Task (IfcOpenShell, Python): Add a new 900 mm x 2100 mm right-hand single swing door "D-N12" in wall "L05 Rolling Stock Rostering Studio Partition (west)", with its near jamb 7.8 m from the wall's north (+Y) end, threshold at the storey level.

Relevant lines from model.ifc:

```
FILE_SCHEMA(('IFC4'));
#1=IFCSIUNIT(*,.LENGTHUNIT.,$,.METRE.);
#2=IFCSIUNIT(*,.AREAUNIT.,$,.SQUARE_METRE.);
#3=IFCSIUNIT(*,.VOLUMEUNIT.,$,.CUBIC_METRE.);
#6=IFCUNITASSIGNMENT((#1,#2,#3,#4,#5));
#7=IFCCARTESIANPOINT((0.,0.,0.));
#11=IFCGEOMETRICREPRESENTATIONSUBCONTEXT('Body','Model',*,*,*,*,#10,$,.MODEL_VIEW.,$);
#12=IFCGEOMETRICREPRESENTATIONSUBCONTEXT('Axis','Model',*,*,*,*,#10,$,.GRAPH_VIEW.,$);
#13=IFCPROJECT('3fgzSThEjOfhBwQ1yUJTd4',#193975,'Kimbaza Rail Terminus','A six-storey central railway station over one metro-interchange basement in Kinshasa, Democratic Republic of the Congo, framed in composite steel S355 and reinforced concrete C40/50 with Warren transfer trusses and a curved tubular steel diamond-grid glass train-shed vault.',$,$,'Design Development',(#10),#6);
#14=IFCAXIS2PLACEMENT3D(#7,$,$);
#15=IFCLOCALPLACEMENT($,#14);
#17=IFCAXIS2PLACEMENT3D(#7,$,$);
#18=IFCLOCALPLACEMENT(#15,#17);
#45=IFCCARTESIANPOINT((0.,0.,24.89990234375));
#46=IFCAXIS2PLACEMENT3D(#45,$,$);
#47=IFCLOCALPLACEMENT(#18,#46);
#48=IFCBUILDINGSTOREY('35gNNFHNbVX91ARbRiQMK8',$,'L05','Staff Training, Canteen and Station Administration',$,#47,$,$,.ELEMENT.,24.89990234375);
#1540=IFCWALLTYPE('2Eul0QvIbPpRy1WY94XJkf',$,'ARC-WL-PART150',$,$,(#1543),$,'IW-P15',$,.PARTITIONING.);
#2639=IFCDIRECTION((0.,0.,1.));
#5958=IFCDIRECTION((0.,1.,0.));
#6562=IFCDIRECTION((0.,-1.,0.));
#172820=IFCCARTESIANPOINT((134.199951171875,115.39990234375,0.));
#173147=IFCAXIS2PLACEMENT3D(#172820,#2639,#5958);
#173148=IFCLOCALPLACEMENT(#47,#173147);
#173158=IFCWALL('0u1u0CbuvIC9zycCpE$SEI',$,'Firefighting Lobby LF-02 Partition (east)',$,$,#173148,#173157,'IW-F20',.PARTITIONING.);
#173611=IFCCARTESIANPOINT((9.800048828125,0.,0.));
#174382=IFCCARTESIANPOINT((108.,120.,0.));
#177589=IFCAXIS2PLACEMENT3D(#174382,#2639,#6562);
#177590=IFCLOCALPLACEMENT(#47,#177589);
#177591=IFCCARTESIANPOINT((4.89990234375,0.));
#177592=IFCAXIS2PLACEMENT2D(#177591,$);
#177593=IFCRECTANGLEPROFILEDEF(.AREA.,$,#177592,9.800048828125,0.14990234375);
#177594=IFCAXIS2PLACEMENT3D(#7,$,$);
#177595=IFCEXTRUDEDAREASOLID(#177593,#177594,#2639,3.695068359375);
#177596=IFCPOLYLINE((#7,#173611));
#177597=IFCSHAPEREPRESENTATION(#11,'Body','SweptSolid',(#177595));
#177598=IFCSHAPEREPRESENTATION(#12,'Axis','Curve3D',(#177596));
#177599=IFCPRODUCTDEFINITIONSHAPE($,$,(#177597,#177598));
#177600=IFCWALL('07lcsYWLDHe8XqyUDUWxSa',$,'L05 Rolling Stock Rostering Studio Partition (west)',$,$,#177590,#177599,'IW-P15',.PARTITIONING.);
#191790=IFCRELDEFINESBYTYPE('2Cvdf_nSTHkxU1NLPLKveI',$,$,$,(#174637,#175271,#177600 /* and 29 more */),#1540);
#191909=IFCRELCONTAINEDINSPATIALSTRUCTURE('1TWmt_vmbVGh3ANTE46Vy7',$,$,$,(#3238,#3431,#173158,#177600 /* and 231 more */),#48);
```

```python
import numpy as np
import ifcopenshell
import ifcopenshell.api.feature
import ifcopenshell.api.geometry
import ifcopenshell.api.root
import ifcopenshell.api.spatial
import ifcopenshell.geom
import ifcopenshell.util.element
import ifcopenshell.util.placement
import ifcopenshell.util.representation
import ifcopenshell.util.shape
import ifcopenshell.util.unit

model = ifcopenshell.open("model.ifc")
unit_scale = ifcopenshell.util.unit.calculate_unit_scale(model)
settings = ifcopenshell.geom.settings()


def volume(element):
    """Net volume in cubic metres, openings subtracted."""
    shape = ifcopenshell.geom.create_shape(settings, element)
    return ifcopenshell.util.shape.get_volume(shape.geometry)


wall = model.by_guid("07lcsYWLDHe8XqyUDUWxSa")
storey = ifcopenshell.util.element.get_container(wall, ifc_class="IfcBuildingStorey")
context = ifcopenshell.util.representation.get_context(model, "Model", "Body", "MODEL_VIEW")
before = volume(wall)

width, height, from_end, sill = 0.9, 2.1, 7.8, 0.0  # metres

# The wall runs along its own X axis, and the end named is its -X end.
wall_shape = ifcopenshell.geom.create_shape(settings, wall)
x, y, z = ifcopenshell.util.shape.get_vertices(wall_shape.geometry).T
start = x.min() + from_end
face, thickness = float(y.min()), float(y.max() - y.min())
wall_matrix = ifcopenshell.util.placement.get_local_placement(wall.ObjectPlacement)
level = ifcopenshell.util.placement.get_local_placement(storey.ObjectPlacement)[2, 3]


def in_wall(x, y):
    """Placement at x, y metres in the wall's axes, at sill height."""
    matrix = wall_matrix.copy()
    matrix[:, 3] = wall_matrix @ np.array([x / unit_scale, y / unit_scale, 0.0, 1.0])
    matrix[2, 3] = level + sill / unit_scale
    return matrix


# Opening: a box that overshoots both wall faces by 50 mm.
opening = ifcopenshell.api.root.create_entity(model, ifc_class="IfcOpeningElement", predefined_type="OPENING")
box = ifcopenshell.api.geometry.add_wall_representation(
    model, context=context, length=width, height=height, thickness=thickness + 0.1
)
ifcopenshell.api.geometry.assign_representation(model, product=opening, representation=box)
ifcopenshell.api.geometry.edit_object_placement(model, product=opening, matrix=in_wall(start, face - 0.05), is_si=False)
ifcopenshell.api.feature.add_feature(model, feature=opening, element=wall)

door = ifcopenshell.api.root.create_entity(model, ifc_class="IfcDoor", name="D-N12", predefined_type="DOOR")
door.OverallWidth, door.OverallHeight = width / unit_scale, height / unit_scale
door.OperationType = "SINGLE_SWING_RIGHT"
body = ifcopenshell.api.geometry.add_door_representation(
    model,
    context=context,
    overall_width=door.OverallWidth,
    overall_height=door.OverallHeight,
    operation_type="SINGLE_SWING_RIGHT",
    lining_properties={"LiningDepth": thickness / unit_scale, "ThresholdDepth": thickness / unit_scale},
)
ifcopenshell.api.geometry.assign_representation(model, product=door, representation=body)
ifcopenshell.api.spatial.assign_container(model, products=[door], relating_structure=storey)
ifcopenshell.api.feature.add_filling(model, opening=opening, element=door)

# The lining spans the wall, so the door starts at the wall face.
ifcopenshell.api.geometry.edit_object_placement(model, product=door, matrix=in_wall(start, face), is_si=False)

after = volume(wall)

print(f"wall volume {before:.3f} -> {after:.3f} m3")

model.write("model_v2.ifc")
```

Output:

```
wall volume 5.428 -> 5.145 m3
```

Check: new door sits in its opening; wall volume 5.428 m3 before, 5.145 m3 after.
